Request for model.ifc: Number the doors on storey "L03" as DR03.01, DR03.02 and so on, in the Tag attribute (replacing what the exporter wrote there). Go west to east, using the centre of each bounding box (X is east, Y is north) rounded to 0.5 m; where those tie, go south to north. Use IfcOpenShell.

First a look at what the model holds.

```python
import ifcopenshell
import ifcopenshell.util.element
import ifcopenshell.util.placement

model = ifcopenshell.open("model.ifc")
print(model.schema)
storey = next(s for s in model.by_type("IfcBuildingStorey") if s.Name == "L03")
doors = [e for e in ifcopenshell.util.element.get_decomposition(storey) if e.is_a("IfcDoor")]
for e in sorted(doors, key=lambda e: e.id()):
    origin = ifcopenshell.util.placement.get_local_placement(e.ObjectPlacement)[:3, 3]
    print(e.id(), e.Tag, e.Name, origin.round(2) + 0.0, sep=" | ")
```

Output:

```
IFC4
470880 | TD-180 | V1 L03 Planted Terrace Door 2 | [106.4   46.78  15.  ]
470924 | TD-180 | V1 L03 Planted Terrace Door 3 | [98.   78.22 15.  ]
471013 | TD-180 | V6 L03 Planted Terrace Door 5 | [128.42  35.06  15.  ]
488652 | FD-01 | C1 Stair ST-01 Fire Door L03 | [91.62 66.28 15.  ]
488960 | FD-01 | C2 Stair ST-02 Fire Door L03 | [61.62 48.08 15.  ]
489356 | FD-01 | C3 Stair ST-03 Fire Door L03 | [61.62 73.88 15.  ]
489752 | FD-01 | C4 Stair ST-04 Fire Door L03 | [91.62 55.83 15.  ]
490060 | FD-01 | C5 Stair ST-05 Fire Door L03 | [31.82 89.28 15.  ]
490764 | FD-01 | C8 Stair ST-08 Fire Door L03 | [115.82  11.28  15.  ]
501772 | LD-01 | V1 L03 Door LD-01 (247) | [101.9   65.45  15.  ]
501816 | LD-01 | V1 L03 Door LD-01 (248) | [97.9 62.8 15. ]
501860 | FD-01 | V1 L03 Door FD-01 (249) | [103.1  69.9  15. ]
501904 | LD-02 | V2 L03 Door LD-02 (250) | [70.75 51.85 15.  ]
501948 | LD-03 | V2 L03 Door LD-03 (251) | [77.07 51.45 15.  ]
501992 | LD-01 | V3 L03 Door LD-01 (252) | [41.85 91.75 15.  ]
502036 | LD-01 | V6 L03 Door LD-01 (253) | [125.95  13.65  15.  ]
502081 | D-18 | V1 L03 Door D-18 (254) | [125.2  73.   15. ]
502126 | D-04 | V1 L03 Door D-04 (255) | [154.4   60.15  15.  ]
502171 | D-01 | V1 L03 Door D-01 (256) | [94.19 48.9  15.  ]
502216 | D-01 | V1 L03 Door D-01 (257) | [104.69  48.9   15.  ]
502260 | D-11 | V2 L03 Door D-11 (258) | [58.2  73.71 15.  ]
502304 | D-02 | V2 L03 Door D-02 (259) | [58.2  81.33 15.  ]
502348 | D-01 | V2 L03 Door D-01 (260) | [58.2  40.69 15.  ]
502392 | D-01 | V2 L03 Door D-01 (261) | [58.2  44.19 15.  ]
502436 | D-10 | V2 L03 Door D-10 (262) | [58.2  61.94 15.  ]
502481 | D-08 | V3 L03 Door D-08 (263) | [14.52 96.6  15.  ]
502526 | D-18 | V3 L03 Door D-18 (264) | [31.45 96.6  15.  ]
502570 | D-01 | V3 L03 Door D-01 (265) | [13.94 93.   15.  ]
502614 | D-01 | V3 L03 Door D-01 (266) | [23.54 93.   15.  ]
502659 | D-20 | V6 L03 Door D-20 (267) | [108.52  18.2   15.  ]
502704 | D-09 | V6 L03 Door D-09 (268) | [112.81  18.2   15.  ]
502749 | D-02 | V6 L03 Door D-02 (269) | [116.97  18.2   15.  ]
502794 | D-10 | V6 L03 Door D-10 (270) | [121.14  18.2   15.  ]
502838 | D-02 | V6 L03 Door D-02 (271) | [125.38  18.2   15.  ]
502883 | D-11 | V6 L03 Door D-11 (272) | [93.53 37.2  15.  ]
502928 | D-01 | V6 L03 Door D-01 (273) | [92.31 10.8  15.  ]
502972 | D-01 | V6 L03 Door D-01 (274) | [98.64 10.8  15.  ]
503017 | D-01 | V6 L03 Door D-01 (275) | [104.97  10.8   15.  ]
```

```python
import ifcopenshell
import ifcopenshell.geom
import ifcopenshell.util.element
import ifcopenshell.util.shape

model = ifcopenshell.open("model.ifc")
settings = ifcopenshell.geom.settings()
settings.set("use-world-coords", True)


def centre(element):
    shape = ifcopenshell.geom.create_shape(settings, element)
    return ifcopenshell.util.shape.get_bbox_centroid(shape.geometry)


storey = next(s for s in model.by_type("IfcBuildingStorey") if s.Name == "L03")
doors = [e for e in ifcopenshell.util.element.get_decomposition(storey) if e.is_a("IfcDoor")]

# Insertion points can sit at a corner or the storey origin, so sort by the geometry (in metres).
centres = {e: centre(e) for e in doors}
doors.sort(key=lambda e: (round(centres[e][0] / 0.5), centres[e][1]))

for i, e in enumerate(doors, start=1):
    number = f"DR03.{i:02d}"
    e.Tag = number
    print(e.id(), number)

model.write("model_rev.ifc")
```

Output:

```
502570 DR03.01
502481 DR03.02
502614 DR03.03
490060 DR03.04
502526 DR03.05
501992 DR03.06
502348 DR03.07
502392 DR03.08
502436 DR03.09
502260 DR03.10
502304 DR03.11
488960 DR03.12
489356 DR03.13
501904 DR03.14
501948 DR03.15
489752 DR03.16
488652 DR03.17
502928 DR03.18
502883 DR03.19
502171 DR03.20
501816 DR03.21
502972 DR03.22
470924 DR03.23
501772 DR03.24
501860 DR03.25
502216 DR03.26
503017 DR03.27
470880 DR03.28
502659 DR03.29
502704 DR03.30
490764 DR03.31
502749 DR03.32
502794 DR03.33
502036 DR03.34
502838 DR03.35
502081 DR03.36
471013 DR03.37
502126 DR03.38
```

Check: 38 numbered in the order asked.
